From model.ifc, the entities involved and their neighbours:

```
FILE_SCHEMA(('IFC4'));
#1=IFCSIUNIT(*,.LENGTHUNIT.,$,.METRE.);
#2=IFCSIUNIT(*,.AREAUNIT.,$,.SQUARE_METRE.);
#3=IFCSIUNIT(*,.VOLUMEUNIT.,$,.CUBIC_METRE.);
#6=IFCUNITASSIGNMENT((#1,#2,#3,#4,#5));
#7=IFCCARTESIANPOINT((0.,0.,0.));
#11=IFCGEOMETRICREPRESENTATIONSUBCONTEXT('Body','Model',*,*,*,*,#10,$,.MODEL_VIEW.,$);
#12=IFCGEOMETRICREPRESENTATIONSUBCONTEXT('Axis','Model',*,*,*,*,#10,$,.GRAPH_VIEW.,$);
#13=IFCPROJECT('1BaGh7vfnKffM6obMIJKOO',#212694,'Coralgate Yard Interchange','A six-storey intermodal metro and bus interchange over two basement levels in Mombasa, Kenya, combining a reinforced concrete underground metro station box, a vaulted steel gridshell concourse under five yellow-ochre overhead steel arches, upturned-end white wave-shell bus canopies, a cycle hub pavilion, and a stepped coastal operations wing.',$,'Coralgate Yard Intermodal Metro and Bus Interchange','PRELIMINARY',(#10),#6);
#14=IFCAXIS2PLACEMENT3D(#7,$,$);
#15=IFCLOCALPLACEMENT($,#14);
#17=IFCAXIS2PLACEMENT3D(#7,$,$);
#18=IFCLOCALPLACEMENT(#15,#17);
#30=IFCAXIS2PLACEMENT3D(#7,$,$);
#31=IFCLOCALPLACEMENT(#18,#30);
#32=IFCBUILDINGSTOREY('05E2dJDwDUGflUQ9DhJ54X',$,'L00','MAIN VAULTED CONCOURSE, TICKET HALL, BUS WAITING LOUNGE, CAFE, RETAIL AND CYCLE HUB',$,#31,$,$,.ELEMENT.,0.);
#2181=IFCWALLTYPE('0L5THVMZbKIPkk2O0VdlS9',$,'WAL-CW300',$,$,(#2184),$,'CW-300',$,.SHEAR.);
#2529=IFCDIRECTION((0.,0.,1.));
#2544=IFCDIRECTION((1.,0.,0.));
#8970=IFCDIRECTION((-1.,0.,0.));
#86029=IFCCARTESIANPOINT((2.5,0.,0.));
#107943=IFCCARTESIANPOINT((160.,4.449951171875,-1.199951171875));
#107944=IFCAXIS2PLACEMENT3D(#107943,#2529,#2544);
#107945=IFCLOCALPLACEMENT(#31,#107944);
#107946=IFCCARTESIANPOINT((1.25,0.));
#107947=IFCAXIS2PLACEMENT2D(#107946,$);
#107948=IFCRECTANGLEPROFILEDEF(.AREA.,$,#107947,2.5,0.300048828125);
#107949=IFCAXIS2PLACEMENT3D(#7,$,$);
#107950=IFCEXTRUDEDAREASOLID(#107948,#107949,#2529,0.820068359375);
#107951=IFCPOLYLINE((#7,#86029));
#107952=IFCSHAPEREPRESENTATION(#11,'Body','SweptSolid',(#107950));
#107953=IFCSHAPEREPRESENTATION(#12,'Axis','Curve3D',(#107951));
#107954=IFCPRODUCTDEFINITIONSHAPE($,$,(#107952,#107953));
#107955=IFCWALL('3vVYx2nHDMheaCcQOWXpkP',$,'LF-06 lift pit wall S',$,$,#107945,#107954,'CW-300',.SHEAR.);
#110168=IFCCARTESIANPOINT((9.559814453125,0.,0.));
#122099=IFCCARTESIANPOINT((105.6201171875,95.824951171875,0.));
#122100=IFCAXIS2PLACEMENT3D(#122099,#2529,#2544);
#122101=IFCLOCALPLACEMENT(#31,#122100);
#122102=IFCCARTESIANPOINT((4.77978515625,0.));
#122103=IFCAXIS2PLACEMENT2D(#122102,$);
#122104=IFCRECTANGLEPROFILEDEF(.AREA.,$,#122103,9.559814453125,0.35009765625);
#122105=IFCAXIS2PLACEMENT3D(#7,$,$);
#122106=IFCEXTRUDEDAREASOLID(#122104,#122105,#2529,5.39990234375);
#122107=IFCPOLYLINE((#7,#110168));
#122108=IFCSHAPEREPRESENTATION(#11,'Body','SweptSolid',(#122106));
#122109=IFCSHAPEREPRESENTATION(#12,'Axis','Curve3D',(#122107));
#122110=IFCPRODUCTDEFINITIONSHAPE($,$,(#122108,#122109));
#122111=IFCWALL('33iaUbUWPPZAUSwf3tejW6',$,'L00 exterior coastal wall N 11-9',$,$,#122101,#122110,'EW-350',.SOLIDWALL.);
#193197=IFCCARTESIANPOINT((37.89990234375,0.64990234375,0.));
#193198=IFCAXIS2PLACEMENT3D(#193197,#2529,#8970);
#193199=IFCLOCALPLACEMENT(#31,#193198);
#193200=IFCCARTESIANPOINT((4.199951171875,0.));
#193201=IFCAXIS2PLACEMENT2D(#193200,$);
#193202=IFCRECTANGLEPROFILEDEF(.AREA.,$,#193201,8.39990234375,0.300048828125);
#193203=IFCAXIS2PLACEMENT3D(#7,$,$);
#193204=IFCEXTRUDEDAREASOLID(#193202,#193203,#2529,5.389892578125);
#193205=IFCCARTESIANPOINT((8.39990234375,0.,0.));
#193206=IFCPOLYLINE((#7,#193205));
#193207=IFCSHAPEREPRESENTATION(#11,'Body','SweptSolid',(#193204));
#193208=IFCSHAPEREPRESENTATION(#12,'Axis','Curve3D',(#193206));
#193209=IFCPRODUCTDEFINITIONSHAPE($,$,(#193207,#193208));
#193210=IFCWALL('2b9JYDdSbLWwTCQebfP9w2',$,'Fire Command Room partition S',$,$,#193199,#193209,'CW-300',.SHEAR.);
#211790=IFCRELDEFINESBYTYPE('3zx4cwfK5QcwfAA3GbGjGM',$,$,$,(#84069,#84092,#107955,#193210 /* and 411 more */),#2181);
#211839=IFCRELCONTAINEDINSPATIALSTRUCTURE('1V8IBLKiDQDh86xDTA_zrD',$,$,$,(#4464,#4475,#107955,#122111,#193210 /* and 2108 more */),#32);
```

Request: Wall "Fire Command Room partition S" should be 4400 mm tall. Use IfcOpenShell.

```python
import ifcopenshell
import ifcopenshell.geom
import ifcopenshell.util.representation
import ifcopenshell.util.shape
import ifcopenshell.util.unit

model = ifcopenshell.open("model.ifc")
unit_scale = ifcopenshell.util.unit.calculate_unit_scale(model)
settings = ifcopenshell.geom.settings()


def volume(element):
    """Net volume in cubic metres, openings subtracted."""
    shape = ifcopenshell.geom.create_shape(settings, element)
    return ifcopenshell.util.shape.get_volume(shape.geometry)


wall = model.by_guid("2b9JYDdSbLWwTCQebfP9w2")
before = volume(wall)

body = ifcopenshell.util.representation.get_representation(wall, "Model", "Body")
solid = body.Items[0]
old_height = solid.Depth
solid.Depth = 4.4 / unit_scale
after = volume(wall)

print(f"height {old_height:g} -> {solid.Depth:g}, volume {before:.3f} -> {after:.3f} m3")

model.write("model-out.ifc")
```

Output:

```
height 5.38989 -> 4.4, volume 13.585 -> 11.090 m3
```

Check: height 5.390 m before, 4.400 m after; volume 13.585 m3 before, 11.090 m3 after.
